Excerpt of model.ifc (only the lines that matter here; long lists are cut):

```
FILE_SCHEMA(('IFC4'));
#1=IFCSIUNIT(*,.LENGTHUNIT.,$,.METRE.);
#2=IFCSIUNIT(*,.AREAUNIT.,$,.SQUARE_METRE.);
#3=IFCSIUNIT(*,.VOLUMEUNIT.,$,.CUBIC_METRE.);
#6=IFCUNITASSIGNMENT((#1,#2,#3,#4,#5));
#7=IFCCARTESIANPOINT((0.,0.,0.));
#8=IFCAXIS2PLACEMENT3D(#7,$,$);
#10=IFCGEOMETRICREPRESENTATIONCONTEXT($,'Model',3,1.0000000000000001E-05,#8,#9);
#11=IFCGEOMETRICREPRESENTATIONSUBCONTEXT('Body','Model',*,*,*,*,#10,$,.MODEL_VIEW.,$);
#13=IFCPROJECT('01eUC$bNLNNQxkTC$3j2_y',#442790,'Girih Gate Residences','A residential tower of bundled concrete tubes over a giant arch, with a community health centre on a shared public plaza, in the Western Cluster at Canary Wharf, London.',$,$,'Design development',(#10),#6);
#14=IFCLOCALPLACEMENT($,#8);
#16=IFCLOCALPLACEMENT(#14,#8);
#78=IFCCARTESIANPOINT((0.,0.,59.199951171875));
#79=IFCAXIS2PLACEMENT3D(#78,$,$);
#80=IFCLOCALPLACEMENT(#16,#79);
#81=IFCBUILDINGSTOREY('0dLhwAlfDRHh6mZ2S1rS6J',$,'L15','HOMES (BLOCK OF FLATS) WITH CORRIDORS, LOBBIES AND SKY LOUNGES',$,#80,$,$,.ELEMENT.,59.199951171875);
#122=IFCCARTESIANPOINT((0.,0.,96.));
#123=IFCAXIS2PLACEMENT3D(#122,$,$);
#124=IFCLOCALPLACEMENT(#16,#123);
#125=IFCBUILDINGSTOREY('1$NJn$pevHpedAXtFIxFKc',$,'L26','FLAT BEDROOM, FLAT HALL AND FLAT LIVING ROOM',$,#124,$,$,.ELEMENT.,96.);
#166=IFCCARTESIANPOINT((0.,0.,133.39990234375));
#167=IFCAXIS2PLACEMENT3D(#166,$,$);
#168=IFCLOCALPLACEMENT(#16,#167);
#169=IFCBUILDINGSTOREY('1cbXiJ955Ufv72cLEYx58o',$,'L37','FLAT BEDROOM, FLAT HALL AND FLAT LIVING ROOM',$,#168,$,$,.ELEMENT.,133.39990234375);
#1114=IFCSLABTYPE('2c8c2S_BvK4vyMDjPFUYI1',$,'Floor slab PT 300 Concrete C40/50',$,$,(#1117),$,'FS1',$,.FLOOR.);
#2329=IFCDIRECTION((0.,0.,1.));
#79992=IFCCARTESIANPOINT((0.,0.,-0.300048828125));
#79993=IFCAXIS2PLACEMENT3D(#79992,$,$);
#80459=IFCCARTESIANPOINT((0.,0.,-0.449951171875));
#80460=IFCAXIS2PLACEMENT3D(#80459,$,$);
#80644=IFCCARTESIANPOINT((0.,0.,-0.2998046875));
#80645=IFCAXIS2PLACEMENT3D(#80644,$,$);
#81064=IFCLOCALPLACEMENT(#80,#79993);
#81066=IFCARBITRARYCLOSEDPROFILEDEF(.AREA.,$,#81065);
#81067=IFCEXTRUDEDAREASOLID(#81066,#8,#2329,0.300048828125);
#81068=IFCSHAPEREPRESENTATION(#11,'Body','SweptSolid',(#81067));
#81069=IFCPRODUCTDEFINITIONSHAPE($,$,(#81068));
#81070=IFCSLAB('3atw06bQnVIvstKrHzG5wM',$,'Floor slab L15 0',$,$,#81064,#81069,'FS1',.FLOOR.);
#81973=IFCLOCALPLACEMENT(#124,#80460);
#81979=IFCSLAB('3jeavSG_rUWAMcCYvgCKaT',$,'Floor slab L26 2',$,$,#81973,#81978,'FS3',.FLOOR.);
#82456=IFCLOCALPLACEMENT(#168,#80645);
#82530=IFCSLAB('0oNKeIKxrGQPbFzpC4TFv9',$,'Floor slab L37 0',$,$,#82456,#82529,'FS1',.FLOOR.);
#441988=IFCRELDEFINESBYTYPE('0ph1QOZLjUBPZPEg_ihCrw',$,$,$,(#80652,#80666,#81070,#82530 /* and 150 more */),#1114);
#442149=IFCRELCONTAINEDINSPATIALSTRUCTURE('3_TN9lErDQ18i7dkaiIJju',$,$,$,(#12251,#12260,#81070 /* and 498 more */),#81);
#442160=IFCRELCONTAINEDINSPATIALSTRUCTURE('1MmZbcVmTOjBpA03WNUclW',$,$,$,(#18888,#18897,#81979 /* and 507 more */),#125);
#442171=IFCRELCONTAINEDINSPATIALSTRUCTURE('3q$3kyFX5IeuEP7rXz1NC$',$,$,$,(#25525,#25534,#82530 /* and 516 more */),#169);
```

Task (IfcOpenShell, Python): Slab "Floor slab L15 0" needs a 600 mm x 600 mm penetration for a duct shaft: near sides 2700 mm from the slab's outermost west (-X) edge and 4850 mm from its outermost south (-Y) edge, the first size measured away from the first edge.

```python
import numpy as np
import ifcopenshell
import ifcopenshell.api.feature
import ifcopenshell.api.geometry
import ifcopenshell.api.root
import ifcopenshell.geom
import ifcopenshell.util.placement
import ifcopenshell.util.representation
import ifcopenshell.util.shape
import ifcopenshell.util.unit

model = ifcopenshell.open("model.ifc")
unit_scale = ifcopenshell.util.unit.calculate_unit_scale(model)
settings = ifcopenshell.geom.settings()


def volume(element):
    """Net volume in cubic metres, openings subtracted."""
    shape = ifcopenshell.geom.create_shape(settings, element)
    return ifcopenshell.util.shape.get_volume(shape.geometry)


slab = model.by_guid("3atw06bQnVIvstKrHzG5wM")
before = volume(slab)

# Extent in the slab's own axes, in metres. The edges named are its -X and -Y sides.
slab_shape = ifcopenshell.geom.create_shape(settings, slab)
vertices = ifcopenshell.util.shape.get_vertices(slab_shape.geometry)
x_min, y_min, bottom = vertices.min(axis=0)
top = vertices[:, 2].max()

opening = ifcopenshell.api.root.create_entity(model, ifc_class="IfcOpeningElement", name="Duct shaft opening", predefined_type="OPENING")
context = ifcopenshell.util.representation.get_context(model, "Model", "Body", "MODEL_VIEW")
width, depth = 0.6, 0.6
outline = [(0.0, 0.0), (width, 0.0), (width, depth), (0.0, depth), (0.0, 0.0)]
# Overshoot both faces by 50 mm so the cut is clean.
shape = ifcopenshell.api.geometry.add_slab_representation(
    model, context=context, depth=top - bottom + 0.1, polyline=outline
)
ifcopenshell.api.geometry.assign_representation(model, product=opening, representation=shape)

matrix = ifcopenshell.util.placement.get_local_placement(slab.ObjectPlacement)
matrix[:, 3] = matrix @ np.append(np.array([x_min + 2.7, y_min + 4.85, bottom - 0.05]) / unit_scale, 1.0)
ifcopenshell.api.geometry.edit_object_placement(model, product=opening, matrix=matrix, is_si=False)
ifcopenshell.api.feature.add_feature(model, feature=opening, element=slab)

after = volume(slab)

print(f"slab volume {before:.3f} -> {after:.3f} m3")

model.write("model_rev.ifc")
```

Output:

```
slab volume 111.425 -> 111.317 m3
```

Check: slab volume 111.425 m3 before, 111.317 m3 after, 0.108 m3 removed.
